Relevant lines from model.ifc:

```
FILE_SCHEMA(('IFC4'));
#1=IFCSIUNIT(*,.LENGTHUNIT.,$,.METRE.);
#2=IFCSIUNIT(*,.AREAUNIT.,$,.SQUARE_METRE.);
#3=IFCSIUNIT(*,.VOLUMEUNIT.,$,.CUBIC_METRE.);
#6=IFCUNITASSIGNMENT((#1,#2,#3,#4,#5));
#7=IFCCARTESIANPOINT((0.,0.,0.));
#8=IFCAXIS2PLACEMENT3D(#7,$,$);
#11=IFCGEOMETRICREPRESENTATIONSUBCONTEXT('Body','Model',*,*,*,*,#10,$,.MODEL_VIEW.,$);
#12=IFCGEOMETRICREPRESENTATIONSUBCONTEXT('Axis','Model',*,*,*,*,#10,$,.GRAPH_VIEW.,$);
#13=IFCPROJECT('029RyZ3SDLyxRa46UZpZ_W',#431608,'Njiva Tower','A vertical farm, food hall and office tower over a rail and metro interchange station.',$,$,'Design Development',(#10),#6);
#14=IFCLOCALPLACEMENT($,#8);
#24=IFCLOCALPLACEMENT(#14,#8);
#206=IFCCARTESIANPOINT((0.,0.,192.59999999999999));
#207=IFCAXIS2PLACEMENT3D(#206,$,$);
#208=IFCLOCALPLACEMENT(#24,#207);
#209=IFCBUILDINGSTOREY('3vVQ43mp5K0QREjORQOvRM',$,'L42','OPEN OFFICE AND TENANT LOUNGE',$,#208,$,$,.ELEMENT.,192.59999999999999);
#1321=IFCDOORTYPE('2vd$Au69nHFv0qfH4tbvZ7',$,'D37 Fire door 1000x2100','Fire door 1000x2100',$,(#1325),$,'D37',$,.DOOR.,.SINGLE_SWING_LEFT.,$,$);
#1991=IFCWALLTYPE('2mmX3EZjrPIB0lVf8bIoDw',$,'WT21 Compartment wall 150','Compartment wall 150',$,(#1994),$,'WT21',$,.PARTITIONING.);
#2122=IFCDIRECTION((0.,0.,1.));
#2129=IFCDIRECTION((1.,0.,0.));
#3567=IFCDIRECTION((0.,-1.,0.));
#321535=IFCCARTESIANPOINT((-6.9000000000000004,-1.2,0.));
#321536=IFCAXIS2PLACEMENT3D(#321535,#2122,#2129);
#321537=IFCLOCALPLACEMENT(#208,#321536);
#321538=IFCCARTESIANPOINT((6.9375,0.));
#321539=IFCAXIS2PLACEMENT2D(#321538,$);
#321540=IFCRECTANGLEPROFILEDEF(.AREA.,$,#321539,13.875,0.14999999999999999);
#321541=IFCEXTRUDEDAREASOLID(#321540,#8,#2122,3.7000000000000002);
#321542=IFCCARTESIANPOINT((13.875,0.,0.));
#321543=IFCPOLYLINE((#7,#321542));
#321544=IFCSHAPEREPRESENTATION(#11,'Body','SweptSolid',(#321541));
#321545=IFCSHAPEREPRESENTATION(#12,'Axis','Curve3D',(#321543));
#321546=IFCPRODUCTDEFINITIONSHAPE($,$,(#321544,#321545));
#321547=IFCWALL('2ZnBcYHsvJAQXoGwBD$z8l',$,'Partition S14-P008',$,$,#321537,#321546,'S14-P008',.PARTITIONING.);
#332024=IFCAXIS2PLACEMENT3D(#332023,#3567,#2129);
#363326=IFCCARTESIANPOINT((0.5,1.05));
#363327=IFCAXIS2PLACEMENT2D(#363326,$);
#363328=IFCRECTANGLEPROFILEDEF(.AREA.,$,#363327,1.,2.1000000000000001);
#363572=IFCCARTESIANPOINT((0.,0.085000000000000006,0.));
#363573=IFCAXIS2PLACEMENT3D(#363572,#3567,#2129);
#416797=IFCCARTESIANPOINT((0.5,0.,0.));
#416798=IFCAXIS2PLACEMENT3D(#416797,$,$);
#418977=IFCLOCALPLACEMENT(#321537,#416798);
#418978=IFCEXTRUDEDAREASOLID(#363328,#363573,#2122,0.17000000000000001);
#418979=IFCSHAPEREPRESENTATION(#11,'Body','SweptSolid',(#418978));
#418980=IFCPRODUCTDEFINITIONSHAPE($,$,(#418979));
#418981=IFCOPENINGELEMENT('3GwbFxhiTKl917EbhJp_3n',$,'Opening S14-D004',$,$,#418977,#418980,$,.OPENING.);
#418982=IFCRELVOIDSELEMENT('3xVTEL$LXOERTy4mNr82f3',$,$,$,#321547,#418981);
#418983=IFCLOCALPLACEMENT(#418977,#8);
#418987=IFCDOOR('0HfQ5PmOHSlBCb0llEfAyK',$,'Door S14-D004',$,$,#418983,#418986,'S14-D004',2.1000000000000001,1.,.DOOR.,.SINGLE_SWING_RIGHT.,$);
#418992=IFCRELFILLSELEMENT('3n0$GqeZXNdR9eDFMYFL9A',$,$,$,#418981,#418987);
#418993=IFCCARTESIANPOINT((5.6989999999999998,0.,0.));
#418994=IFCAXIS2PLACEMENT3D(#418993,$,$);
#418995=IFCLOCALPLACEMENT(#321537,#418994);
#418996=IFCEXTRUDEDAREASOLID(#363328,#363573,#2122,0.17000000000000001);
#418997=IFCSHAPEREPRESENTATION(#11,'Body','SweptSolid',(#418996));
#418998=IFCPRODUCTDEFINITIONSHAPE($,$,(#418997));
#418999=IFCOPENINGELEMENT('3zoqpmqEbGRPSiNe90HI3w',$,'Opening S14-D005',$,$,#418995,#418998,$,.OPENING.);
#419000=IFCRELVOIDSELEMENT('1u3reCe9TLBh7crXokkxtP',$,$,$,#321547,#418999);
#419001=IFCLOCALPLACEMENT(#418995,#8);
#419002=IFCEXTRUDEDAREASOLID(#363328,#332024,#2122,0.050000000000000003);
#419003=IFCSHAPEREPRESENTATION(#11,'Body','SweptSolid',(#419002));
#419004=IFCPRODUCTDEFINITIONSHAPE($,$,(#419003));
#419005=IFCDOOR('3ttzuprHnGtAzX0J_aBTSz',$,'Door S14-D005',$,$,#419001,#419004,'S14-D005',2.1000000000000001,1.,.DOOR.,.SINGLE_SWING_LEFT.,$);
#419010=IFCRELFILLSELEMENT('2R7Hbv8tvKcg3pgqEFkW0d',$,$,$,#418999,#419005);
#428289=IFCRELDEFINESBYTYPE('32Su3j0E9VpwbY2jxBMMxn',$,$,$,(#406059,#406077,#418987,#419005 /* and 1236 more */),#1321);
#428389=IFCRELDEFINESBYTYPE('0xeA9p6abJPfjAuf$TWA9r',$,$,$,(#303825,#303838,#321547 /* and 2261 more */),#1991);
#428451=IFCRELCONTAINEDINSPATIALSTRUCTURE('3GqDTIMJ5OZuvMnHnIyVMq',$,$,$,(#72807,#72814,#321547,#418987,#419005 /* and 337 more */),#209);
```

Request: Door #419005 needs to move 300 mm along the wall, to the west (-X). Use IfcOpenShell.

```python
import ifcopenshell
import ifcopenshell.api.geometry
import ifcopenshell.util.placement

model = ifcopenshell.open("model.ifc")

door = model.by_guid("3ttzuprHnGtAzX0J_aBTSz")
opening = door.FillsVoids[0].RelatingOpeningElement
wall = opening.VoidsElements[0].RelatingBuildingElement

wall_matrix = ifcopenshell.util.placement.get_local_placement(wall.ObjectPlacement)
shift = wall_matrix[:3, 0] * -0.3
before = ifcopenshell.util.placement.get_local_placement(door.ObjectPlacement)[:3, 3].copy()

# The door is placed relative to its opening, so it follows when the opening moves.
matrix = ifcopenshell.util.placement.get_local_placement(opening.ObjectPlacement)
matrix[:3, 3] += shift
ifcopenshell.api.geometry.edit_object_placement(
    model, product=opening, matrix=matrix, is_si=False, should_transform_children=True
)

after = ifcopenshell.util.placement.get_local_placement(door.ObjectPlacement)[:3, 3]
print("door moved by", (after - before).round(3) + 0.0)

model.write("model_v2.ifc")
```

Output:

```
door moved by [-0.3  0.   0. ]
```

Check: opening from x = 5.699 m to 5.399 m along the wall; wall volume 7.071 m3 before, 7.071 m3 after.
